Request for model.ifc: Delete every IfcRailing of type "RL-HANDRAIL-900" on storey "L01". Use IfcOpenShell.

First a look at what the model holds.

```python
import ifcopenshell
import ifcopenshell.util.element

model = ifcopenshell.open("model.ifc")
print(model.schema)
storey = next(s for s in model.by_type("IfcBuildingStorey") if s.Name == "L01")
railings = [e for e in ifcopenshell.util.element.get_decomposition(storey) if e.is_a("IfcRailing")]
seen = {}
for e in railings:
    element_type = ifcopenshell.util.element.get_type(e)
    name = element_type.Name if element_type not in (None, e) else None
    seen[name] = seen.get(name, 0) + 1
for name, count in sorted(seen.items(), key=str):
    print(count, "x", name)
```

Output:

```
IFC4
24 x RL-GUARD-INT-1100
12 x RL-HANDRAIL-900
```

```python
import ifcopenshell
import ifcopenshell.api.root
import ifcopenshell.util.element

model = ifcopenshell.open("model.ifc")

storey = next(s for s in model.by_type("IfcBuildingStorey") if s.Name == "L01")
railings = [e for e in ifcopenshell.util.element.get_decomposition(storey) if e.is_a("IfcRailing")]
targets = [e for e in railings if (t := ifcopenshell.util.element.get_type(e)) not in (None, e) and t.Name == "RL-HANDRAIL-900"]

for e in targets:
    ifcopenshell.api.root.remove_product(model, product=e)
print(len(targets), "removed")

model.write("model_v2.ifc")
```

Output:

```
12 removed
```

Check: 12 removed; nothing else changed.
